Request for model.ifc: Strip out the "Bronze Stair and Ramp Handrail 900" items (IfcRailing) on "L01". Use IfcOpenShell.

First a look at what the model holds.

```python
import ifcopenshell
import ifcopenshell.util.element

model = ifcopenshell.open("model.ifc")
print(model.schema)
storey = next(s for s in model.by_type("IfcBuildingStorey") if s.Name == "L01")
railings = [e for e in ifcopenshell.util.element.get_decomposition(storey) if e.is_a("IfcRailing")]
seen = {}
for e in railings:
    element_type = ifcopenshell.util.element.get_type(e)
    name = element_type.Name if element_type not in (None, e) else None
    seen[name] = seen.get(name, 0) + 1
for name, count in sorted(seen.items(), key=str):
    print(count, "x", name)
```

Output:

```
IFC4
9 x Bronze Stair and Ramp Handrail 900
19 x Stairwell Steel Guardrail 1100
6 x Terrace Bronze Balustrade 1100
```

```python
import ifcopenshell
import ifcopenshell.api.root
import ifcopenshell.util.element

model = ifcopenshell.open("model.ifc")

storey = next(s for s in model.by_type("IfcBuildingStorey") if s.Name == "L01")
railings = [e for e in ifcopenshell.util.element.get_decomposition(storey) if e.is_a("IfcRailing")]
targets = [e for e in railings if (t := ifcopenshell.util.element.get_type(e)) not in (None, e) and t.Name == "Bronze Stair and Ramp Handrail 900"]

for e in targets:
    ifcopenshell.api.root.remove_product(model, product=e)
print(len(targets), "removed")

model.write("model-out.ifc")
```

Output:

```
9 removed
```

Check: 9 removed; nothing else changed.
